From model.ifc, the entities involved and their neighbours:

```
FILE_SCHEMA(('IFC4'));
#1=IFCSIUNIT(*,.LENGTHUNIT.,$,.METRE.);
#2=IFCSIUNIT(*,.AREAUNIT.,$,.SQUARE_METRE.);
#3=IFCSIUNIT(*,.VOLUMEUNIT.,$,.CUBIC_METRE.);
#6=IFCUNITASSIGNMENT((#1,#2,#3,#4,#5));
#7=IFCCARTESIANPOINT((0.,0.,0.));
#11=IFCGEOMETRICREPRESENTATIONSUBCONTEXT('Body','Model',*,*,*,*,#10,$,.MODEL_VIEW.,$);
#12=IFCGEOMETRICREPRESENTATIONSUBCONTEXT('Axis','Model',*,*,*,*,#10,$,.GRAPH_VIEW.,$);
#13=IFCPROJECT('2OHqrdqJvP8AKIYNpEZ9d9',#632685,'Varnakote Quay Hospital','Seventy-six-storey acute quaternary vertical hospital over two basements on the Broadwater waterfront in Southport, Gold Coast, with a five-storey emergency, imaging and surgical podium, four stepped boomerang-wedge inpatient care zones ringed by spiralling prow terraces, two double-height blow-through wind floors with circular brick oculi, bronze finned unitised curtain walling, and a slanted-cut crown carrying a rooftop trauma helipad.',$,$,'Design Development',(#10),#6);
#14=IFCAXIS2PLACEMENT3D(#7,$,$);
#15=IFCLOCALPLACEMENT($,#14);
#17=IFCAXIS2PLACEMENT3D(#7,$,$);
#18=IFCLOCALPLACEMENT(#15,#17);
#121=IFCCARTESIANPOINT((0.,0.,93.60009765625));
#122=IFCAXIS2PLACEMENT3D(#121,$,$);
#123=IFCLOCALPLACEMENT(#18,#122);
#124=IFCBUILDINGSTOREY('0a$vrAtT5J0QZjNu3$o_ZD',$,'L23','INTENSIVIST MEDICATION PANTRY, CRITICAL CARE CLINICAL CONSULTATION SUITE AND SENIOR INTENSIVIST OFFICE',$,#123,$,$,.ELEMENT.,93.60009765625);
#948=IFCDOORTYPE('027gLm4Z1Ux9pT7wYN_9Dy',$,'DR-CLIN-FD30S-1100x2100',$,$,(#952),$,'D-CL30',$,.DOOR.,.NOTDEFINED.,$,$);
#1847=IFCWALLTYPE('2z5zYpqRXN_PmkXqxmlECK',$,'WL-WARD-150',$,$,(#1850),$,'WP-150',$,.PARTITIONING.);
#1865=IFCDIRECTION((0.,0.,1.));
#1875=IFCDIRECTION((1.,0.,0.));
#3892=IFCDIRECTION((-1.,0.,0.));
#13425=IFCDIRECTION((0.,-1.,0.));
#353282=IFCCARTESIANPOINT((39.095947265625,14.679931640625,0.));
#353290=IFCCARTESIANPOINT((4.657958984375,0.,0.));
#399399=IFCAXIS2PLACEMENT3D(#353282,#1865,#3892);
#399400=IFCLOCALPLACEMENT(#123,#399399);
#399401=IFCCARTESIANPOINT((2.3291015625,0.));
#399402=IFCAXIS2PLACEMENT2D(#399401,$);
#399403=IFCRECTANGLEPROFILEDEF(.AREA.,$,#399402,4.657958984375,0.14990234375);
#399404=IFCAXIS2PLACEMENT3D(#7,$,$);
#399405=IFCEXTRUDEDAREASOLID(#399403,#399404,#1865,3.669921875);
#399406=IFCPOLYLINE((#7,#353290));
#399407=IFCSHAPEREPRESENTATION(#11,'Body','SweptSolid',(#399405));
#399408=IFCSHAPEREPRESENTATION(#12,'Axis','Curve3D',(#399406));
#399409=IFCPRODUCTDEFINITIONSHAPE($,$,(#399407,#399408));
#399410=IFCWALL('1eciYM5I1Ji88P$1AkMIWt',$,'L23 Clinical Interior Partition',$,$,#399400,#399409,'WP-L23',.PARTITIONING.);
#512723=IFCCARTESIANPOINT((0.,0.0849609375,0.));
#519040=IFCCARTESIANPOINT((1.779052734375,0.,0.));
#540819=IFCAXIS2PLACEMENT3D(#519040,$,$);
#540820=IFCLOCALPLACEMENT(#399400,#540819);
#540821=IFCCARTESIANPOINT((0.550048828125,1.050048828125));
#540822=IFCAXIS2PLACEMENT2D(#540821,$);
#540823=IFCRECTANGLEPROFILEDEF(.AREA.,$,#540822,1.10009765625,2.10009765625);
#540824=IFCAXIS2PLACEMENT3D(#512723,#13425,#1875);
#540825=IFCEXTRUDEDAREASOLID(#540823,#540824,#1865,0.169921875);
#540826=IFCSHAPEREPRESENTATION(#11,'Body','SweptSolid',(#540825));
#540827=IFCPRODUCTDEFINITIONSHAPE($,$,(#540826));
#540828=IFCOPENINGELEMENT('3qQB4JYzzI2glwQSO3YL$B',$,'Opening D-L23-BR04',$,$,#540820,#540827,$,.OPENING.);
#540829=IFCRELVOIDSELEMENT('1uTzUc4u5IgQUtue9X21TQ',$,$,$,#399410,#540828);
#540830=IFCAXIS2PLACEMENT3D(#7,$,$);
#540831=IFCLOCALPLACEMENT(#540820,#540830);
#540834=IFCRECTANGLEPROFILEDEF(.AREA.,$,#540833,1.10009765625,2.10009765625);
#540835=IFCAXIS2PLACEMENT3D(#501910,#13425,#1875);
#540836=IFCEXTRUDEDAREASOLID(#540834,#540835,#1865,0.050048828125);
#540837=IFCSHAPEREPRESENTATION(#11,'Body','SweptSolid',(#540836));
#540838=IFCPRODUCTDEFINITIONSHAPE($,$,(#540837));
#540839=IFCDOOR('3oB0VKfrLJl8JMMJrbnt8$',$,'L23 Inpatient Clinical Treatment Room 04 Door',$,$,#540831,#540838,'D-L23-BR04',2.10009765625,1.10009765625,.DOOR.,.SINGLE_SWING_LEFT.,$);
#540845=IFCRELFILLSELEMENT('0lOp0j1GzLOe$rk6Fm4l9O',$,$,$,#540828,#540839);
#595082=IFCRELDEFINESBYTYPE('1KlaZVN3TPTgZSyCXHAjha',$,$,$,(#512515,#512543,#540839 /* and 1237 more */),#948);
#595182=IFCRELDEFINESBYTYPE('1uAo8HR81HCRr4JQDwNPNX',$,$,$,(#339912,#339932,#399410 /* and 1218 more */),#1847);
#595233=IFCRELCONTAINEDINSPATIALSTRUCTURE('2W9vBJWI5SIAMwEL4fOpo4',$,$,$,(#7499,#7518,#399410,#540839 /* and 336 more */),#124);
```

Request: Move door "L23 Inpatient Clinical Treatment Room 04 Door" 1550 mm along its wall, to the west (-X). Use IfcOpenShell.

```python
import ifcopenshell
import ifcopenshell.api.geometry
import ifcopenshell.util.placement
import ifcopenshell.util.unit

model = ifcopenshell.open("model.ifc")
unit_scale = ifcopenshell.util.unit.calculate_unit_scale(model)

door = model.by_guid("3oB0VKfrLJl8JMMJrbnt8$")
opening = door.FillsVoids[0].RelatingOpeningElement
wall = opening.VoidsElements[0].RelatingBuildingElement

wall_matrix = ifcopenshell.util.placement.get_local_placement(wall.ObjectPlacement)
shift = wall_matrix[:3, 0] * 1.55 / unit_scale
before = ifcopenshell.util.placement.get_local_placement(door.ObjectPlacement)[:3, 3].copy()

# The door is placed relative to its opening, so it follows when the opening moves.
matrix = ifcopenshell.util.placement.get_local_placement(opening.ObjectPlacement)
matrix[:3, 3] += shift
ifcopenshell.api.geometry.edit_object_placement(
    model, product=opening, matrix=matrix, is_si=False, should_transform_children=True
)

after = ifcopenshell.util.placement.get_local_placement(door.ObjectPlacement)[:3, 3]
print("door moved by", (after - before).round(3) + 0.0)

model.write("model-out.ifc")
```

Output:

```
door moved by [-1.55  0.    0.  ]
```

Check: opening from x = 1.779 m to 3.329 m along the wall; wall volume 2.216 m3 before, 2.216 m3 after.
